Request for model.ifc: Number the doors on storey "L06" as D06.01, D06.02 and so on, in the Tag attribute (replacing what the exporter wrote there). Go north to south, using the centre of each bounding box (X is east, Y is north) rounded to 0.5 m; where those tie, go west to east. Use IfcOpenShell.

First a look at what the model holds.

```python
import ifcopenshell
import ifcopenshell.util.element
import ifcopenshell.util.placement

model = ifcopenshell.open("model.ifc")
print(model.schema)
storey = next(s for s in model.by_type("IfcBuildingStorey") if s.Name == "L06")
doors = [e for e in ifcopenshell.util.element.get_decomposition(storey) if e.is_a("IfcDoor")]
for e in sorted(doors, key=lambda e: e.id()):
    origin = ifcopenshell.util.placement.get_local_placement(e.ObjectPlacement)[:3, 3]
    print(e.id(), e.Tag, e.Name, origin.round(2) + 0.0, sep=" | ")
```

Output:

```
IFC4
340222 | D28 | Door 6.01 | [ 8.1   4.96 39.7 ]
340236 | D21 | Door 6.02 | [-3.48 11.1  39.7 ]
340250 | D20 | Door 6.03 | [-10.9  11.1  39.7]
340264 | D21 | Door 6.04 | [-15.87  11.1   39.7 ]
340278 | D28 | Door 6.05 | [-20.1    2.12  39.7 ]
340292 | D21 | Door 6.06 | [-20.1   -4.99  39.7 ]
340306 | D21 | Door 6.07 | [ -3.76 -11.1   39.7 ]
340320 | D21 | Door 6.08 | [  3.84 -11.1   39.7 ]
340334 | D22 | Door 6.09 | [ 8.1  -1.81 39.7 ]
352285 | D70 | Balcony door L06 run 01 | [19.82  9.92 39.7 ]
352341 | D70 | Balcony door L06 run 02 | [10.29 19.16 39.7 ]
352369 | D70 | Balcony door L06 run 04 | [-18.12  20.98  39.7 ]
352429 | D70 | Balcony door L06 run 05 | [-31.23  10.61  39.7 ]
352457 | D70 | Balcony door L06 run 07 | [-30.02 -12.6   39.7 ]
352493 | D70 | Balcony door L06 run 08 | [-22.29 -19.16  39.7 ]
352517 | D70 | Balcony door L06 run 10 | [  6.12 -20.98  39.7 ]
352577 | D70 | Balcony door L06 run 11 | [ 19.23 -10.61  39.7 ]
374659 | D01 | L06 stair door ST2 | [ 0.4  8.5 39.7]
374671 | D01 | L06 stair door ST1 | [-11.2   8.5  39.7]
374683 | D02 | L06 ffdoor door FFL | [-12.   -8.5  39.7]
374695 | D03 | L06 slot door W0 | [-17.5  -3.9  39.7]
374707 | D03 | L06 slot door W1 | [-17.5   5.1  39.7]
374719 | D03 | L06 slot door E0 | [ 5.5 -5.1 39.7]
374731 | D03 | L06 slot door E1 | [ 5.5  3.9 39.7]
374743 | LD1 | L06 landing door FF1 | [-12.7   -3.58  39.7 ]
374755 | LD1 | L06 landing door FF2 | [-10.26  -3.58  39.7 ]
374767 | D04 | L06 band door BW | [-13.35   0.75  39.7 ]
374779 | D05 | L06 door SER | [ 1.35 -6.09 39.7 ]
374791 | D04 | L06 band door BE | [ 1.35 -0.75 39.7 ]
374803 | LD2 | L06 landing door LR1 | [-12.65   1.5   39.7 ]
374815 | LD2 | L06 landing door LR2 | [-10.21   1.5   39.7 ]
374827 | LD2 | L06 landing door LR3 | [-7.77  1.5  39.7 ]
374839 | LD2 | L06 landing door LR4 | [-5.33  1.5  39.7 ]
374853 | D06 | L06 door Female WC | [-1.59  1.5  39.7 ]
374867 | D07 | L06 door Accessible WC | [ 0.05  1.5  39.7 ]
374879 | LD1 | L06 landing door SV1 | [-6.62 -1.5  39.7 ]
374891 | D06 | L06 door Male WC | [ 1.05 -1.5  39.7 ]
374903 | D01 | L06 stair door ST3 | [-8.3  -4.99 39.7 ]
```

```python
import ifcopenshell
import ifcopenshell.geom
import ifcopenshell.util.element
import ifcopenshell.util.shape

model = ifcopenshell.open("model.ifc")
settings = ifcopenshell.geom.settings()
settings.set("use-world-coords", True)


def centre(element):
    shape = ifcopenshell.geom.create_shape(settings, element)
    return ifcopenshell.util.shape.get_bbox_centroid(shape.geometry)


storey = next(s for s in model.by_type("IfcBuildingStorey") if s.Name == "L06")
doors = [e for e in ifcopenshell.util.element.get_decomposition(storey) if e.is_a("IfcDoor")]

# Insertion points can sit at a corner or the storey origin, so sort by the geometry (in metres).
centres = {e: centre(e) for e in doors}
doors.sort(key=lambda e: (-round(centres[e][1] / 0.5), centres[e][0]))

for i, e in enumerate(doors, start=1):
    number = f"D06.{i:02d}"
    e.Tag = number
    print(e.id(), number)

model.write("model_v2.ifc")
```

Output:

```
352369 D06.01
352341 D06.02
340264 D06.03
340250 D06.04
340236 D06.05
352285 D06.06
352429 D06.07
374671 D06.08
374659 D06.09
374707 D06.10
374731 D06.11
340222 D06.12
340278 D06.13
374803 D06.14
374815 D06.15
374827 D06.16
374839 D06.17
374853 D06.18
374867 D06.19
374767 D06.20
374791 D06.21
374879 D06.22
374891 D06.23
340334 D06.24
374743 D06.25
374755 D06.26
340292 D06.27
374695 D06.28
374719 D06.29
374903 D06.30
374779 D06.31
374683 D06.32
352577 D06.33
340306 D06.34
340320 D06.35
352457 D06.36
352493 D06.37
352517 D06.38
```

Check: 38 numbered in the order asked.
